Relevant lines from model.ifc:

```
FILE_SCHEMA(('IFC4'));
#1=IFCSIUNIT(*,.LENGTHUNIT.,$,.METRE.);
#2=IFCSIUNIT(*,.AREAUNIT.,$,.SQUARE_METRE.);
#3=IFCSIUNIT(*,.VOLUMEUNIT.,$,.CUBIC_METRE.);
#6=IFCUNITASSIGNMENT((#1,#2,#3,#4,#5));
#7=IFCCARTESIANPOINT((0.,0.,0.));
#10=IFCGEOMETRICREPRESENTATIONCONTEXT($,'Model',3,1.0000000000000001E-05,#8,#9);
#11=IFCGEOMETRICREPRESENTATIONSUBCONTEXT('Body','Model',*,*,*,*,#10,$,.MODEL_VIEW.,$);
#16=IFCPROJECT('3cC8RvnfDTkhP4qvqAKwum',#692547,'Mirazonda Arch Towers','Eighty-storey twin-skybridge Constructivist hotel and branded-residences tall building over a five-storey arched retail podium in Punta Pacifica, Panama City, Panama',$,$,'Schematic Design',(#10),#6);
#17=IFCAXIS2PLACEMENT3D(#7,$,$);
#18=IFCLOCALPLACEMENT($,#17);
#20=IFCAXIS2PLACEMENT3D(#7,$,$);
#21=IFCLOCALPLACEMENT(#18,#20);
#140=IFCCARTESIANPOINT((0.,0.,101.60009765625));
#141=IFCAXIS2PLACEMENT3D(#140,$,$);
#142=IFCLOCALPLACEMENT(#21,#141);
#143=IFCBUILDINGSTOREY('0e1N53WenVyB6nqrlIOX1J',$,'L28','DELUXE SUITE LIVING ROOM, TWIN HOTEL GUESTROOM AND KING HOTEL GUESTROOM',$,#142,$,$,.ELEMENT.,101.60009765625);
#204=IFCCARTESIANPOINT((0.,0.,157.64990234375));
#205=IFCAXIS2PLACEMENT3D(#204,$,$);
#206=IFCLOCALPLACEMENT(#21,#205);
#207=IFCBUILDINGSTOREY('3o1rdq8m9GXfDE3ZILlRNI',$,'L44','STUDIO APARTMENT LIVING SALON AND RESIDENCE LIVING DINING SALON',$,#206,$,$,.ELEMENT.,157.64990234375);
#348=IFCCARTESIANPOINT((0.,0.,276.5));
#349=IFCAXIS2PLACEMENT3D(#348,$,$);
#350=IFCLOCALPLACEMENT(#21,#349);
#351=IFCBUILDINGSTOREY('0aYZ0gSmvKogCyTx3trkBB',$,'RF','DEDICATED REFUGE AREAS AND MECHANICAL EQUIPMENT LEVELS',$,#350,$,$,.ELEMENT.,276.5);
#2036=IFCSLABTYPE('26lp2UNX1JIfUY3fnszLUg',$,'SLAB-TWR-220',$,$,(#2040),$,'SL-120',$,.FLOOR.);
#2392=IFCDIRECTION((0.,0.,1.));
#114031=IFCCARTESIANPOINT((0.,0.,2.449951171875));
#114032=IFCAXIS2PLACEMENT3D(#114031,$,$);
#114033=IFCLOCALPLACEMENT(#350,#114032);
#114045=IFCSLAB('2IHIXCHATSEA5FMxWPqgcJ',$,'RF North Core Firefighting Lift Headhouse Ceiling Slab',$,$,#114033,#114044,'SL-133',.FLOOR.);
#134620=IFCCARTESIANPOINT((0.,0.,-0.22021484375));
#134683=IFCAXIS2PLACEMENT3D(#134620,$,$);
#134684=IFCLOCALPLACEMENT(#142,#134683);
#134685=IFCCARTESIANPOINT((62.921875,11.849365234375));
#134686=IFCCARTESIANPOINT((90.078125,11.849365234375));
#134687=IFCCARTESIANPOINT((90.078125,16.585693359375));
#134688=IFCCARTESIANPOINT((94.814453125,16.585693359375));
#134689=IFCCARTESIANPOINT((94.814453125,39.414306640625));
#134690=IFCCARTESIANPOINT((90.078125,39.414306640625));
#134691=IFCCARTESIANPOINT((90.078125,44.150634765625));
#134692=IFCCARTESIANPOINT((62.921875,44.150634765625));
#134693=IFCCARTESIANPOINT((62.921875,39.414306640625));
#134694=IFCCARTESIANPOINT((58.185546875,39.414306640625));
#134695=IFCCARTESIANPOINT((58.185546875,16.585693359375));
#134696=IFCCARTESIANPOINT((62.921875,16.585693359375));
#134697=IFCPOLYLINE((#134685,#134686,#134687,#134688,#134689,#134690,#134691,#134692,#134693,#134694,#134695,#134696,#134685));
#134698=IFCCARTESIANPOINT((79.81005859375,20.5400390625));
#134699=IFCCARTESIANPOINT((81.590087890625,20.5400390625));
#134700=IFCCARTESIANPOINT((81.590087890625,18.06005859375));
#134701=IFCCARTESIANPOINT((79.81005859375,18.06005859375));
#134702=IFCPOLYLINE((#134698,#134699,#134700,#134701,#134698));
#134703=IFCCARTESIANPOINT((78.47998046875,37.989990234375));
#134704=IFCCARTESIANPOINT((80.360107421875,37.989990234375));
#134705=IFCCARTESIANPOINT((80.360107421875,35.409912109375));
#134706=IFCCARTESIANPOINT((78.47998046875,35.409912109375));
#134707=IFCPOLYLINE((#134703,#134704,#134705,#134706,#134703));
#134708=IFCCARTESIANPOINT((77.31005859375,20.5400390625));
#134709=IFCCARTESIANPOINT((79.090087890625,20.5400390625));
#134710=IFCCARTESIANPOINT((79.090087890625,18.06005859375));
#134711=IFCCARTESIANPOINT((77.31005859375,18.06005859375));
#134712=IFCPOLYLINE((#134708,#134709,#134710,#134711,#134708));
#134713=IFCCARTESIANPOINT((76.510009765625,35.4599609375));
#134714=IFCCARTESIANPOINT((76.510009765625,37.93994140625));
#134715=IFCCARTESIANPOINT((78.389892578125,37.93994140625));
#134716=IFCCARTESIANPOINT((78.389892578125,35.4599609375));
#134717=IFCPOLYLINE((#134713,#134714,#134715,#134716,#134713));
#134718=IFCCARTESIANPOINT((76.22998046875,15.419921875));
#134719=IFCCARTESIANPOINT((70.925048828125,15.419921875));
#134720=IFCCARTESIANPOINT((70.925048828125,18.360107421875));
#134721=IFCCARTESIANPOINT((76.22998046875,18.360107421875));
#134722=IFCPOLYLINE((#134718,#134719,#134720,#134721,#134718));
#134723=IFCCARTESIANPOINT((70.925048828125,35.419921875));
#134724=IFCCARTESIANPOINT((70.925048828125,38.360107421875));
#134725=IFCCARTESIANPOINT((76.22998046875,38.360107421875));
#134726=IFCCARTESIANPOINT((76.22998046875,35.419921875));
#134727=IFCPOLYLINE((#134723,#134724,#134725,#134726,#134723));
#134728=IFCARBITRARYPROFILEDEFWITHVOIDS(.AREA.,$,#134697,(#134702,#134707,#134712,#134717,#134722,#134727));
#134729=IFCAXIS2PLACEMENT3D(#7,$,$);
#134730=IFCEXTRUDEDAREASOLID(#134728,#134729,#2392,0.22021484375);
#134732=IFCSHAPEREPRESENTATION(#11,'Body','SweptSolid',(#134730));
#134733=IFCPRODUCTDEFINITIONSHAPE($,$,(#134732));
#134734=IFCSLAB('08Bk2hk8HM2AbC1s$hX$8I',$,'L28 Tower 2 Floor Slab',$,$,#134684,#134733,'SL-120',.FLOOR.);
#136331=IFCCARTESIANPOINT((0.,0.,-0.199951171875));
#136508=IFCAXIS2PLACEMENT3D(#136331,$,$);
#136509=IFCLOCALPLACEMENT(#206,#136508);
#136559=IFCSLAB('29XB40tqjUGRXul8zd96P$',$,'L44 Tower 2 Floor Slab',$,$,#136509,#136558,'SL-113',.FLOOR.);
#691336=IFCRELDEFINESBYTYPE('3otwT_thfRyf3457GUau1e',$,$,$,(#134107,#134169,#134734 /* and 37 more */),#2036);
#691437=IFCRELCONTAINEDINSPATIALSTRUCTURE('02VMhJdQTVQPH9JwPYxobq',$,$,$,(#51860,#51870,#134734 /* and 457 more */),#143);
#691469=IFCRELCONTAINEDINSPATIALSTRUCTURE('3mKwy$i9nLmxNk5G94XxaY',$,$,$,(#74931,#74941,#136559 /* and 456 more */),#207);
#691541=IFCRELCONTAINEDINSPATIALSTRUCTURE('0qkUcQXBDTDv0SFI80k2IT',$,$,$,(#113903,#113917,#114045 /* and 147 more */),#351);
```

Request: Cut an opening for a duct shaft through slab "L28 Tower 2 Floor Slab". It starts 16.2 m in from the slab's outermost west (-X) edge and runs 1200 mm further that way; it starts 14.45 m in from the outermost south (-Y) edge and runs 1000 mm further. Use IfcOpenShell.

```python
import numpy as np
import ifcopenshell
import ifcopenshell.api.feature
import ifcopenshell.api.geometry
import ifcopenshell.api.root
import ifcopenshell.geom
import ifcopenshell.util.placement
import ifcopenshell.util.representation
import ifcopenshell.util.shape
import ifcopenshell.util.unit

model = ifcopenshell.open("model.ifc")
unit_scale = ifcopenshell.util.unit.calculate_unit_scale(model)
settings = ifcopenshell.geom.settings()


def volume(element):
    """Net volume in cubic metres, openings subtracted."""
    shape = ifcopenshell.geom.create_shape(settings, element)
    return ifcopenshell.util.shape.get_volume(shape.geometry)


slab = model.by_guid("08Bk2hk8HM2AbC1s$hX$8I")
before = volume(slab)

# Extent in the slab's own axes, in metres. The edges named are its -X and -Y sides.
slab_shape = ifcopenshell.geom.create_shape(settings, slab)
vertices = ifcopenshell.util.shape.get_vertices(slab_shape.geometry)
x_min, y_min, bottom = vertices.min(axis=0)
top = vertices[:, 2].max()

opening = ifcopenshell.api.root.create_entity(model, ifc_class="IfcOpeningElement", name="Duct shaft opening", predefined_type="OPENING")
context = ifcopenshell.util.representation.get_context(model, "Model", "Body", "MODEL_VIEW")
width, depth = 1.2, 1
outline = [(0.0, 0.0), (width, 0.0), (width, depth), (0.0, depth), (0.0, 0.0)]
# Overshoot both faces by 50 mm so the cut is clean.
shape = ifcopenshell.api.geometry.add_slab_representation(
    model, context=context, depth=top - bottom + 0.1, polyline=outline
)
ifcopenshell.api.geometry.assign_representation(model, product=opening, representation=shape)

matrix = ifcopenshell.util.placement.get_local_placement(slab.ObjectPlacement)
matrix[:, 3] = matrix @ np.append(np.array([x_min + 16.2, y_min + 14.45, bottom - 0.05]) / unit_scale, 1.0)
ifcopenshell.api.geometry.edit_object_placement(model, product=opening, matrix=matrix, is_si=False)
ifcopenshell.api.feature.add_feature(model, feature=opening, element=slab)

after = volume(slab)

print(f"slab volume {before:.3f} -> {after:.3f} m3")

model.write("model_updated.ifc")
```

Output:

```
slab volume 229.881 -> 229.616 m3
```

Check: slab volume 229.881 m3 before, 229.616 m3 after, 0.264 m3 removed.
